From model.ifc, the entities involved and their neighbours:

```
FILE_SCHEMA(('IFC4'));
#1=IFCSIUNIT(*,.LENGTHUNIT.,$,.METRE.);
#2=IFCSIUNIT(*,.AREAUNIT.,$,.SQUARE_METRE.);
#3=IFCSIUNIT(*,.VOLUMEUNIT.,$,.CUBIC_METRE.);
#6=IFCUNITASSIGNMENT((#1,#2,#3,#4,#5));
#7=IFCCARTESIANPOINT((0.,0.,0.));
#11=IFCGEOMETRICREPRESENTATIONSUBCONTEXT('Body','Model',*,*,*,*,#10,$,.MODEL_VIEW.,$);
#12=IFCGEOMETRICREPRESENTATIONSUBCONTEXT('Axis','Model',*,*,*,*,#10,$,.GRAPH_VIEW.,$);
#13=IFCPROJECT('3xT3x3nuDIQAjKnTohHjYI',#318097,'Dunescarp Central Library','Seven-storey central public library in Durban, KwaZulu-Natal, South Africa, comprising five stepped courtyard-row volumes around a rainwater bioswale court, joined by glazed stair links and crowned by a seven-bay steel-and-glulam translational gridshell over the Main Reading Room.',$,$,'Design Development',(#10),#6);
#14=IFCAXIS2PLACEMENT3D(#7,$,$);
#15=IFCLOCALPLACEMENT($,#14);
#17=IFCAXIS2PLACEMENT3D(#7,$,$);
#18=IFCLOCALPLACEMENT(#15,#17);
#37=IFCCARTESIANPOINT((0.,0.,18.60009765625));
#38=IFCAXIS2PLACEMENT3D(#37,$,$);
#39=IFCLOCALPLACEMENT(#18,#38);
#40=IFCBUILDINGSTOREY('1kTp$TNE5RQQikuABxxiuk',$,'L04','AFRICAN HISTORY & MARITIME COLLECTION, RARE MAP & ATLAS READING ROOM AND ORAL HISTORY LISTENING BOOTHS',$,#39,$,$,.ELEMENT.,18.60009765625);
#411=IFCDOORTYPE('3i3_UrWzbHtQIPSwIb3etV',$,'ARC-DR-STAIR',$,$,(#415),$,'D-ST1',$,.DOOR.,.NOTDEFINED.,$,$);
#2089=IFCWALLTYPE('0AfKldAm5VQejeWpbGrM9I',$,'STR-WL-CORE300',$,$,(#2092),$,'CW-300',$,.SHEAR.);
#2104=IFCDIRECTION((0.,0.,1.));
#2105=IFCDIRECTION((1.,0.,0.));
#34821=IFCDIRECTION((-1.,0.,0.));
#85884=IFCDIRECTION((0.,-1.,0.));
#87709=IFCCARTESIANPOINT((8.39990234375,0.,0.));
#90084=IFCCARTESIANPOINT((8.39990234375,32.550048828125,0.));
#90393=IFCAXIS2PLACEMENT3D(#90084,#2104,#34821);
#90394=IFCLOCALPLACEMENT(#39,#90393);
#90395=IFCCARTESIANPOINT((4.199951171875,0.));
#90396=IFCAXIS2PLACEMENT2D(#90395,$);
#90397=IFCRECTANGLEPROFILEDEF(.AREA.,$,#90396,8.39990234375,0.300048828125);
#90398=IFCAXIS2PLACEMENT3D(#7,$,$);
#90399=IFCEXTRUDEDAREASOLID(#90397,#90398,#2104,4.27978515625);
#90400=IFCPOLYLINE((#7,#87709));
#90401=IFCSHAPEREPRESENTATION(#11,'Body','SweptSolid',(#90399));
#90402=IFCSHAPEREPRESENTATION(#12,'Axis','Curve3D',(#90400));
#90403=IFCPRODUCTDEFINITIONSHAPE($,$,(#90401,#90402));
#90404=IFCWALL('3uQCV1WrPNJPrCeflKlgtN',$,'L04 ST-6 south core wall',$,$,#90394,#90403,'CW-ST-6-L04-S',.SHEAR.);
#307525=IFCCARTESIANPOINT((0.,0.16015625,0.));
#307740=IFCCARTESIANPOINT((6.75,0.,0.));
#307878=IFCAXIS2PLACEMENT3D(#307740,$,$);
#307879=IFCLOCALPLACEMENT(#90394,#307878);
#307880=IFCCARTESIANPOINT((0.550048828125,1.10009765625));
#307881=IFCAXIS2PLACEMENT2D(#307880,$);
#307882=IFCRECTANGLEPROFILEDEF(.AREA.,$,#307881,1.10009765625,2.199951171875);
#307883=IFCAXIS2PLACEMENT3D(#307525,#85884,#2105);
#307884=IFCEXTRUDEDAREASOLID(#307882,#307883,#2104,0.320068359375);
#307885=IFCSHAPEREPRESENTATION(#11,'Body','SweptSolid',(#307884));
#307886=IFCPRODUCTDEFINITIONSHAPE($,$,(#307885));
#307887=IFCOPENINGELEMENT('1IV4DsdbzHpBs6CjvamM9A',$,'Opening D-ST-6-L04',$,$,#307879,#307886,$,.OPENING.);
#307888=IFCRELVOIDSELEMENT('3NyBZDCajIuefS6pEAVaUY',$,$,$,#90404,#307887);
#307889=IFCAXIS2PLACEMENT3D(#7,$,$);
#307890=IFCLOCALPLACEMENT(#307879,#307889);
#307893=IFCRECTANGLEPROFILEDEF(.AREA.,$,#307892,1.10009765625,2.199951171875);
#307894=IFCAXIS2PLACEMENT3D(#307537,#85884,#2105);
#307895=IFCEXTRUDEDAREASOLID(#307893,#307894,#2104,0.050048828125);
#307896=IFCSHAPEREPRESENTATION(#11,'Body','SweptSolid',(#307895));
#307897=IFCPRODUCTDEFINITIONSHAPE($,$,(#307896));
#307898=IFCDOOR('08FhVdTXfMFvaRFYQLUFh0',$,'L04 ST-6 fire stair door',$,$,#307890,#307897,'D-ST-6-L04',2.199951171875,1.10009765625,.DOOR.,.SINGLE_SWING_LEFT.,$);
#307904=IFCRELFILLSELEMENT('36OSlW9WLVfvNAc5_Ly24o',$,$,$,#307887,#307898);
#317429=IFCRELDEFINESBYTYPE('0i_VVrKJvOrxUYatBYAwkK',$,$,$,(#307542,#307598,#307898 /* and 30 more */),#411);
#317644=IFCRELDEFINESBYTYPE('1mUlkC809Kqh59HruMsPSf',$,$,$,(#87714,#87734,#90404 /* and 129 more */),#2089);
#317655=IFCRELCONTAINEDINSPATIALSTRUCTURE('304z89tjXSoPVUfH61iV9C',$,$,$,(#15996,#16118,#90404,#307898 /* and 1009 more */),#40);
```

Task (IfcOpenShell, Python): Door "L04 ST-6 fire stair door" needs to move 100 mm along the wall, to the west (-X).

```python
import ifcopenshell
import ifcopenshell.api.geometry
import ifcopenshell.util.placement
import ifcopenshell.util.unit

model = ifcopenshell.open("model.ifc")
unit_scale = ifcopenshell.util.unit.calculate_unit_scale(model)

door = model.by_guid("08FhVdTXfMFvaRFYQLUFh0")
opening = door.FillsVoids[0].RelatingOpeningElement
wall = opening.VoidsElements[0].RelatingBuildingElement

wall_matrix = ifcopenshell.util.placement.get_local_placement(wall.ObjectPlacement)
shift = wall_matrix[:3, 0] * 0.1 / unit_scale
before = ifcopenshell.util.placement.get_local_placement(door.ObjectPlacement)[:3, 3].copy()

# The door is placed relative to its opening, so it follows when the opening moves.
matrix = ifcopenshell.util.placement.get_local_placement(opening.ObjectPlacement)
matrix[:3, 3] += shift
ifcopenshell.api.geometry.edit_object_placement(
    model, product=opening, matrix=matrix, is_si=False, should_transform_children=True
)

after = ifcopenshell.util.placement.get_local_placement(door.ObjectPlacement)[:3, 3]
print("door moved by", (after - before).round(3) + 0.0)

model.write("model_edited.ifc")
```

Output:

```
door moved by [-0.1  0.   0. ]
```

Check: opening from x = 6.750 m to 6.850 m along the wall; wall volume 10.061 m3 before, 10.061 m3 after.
